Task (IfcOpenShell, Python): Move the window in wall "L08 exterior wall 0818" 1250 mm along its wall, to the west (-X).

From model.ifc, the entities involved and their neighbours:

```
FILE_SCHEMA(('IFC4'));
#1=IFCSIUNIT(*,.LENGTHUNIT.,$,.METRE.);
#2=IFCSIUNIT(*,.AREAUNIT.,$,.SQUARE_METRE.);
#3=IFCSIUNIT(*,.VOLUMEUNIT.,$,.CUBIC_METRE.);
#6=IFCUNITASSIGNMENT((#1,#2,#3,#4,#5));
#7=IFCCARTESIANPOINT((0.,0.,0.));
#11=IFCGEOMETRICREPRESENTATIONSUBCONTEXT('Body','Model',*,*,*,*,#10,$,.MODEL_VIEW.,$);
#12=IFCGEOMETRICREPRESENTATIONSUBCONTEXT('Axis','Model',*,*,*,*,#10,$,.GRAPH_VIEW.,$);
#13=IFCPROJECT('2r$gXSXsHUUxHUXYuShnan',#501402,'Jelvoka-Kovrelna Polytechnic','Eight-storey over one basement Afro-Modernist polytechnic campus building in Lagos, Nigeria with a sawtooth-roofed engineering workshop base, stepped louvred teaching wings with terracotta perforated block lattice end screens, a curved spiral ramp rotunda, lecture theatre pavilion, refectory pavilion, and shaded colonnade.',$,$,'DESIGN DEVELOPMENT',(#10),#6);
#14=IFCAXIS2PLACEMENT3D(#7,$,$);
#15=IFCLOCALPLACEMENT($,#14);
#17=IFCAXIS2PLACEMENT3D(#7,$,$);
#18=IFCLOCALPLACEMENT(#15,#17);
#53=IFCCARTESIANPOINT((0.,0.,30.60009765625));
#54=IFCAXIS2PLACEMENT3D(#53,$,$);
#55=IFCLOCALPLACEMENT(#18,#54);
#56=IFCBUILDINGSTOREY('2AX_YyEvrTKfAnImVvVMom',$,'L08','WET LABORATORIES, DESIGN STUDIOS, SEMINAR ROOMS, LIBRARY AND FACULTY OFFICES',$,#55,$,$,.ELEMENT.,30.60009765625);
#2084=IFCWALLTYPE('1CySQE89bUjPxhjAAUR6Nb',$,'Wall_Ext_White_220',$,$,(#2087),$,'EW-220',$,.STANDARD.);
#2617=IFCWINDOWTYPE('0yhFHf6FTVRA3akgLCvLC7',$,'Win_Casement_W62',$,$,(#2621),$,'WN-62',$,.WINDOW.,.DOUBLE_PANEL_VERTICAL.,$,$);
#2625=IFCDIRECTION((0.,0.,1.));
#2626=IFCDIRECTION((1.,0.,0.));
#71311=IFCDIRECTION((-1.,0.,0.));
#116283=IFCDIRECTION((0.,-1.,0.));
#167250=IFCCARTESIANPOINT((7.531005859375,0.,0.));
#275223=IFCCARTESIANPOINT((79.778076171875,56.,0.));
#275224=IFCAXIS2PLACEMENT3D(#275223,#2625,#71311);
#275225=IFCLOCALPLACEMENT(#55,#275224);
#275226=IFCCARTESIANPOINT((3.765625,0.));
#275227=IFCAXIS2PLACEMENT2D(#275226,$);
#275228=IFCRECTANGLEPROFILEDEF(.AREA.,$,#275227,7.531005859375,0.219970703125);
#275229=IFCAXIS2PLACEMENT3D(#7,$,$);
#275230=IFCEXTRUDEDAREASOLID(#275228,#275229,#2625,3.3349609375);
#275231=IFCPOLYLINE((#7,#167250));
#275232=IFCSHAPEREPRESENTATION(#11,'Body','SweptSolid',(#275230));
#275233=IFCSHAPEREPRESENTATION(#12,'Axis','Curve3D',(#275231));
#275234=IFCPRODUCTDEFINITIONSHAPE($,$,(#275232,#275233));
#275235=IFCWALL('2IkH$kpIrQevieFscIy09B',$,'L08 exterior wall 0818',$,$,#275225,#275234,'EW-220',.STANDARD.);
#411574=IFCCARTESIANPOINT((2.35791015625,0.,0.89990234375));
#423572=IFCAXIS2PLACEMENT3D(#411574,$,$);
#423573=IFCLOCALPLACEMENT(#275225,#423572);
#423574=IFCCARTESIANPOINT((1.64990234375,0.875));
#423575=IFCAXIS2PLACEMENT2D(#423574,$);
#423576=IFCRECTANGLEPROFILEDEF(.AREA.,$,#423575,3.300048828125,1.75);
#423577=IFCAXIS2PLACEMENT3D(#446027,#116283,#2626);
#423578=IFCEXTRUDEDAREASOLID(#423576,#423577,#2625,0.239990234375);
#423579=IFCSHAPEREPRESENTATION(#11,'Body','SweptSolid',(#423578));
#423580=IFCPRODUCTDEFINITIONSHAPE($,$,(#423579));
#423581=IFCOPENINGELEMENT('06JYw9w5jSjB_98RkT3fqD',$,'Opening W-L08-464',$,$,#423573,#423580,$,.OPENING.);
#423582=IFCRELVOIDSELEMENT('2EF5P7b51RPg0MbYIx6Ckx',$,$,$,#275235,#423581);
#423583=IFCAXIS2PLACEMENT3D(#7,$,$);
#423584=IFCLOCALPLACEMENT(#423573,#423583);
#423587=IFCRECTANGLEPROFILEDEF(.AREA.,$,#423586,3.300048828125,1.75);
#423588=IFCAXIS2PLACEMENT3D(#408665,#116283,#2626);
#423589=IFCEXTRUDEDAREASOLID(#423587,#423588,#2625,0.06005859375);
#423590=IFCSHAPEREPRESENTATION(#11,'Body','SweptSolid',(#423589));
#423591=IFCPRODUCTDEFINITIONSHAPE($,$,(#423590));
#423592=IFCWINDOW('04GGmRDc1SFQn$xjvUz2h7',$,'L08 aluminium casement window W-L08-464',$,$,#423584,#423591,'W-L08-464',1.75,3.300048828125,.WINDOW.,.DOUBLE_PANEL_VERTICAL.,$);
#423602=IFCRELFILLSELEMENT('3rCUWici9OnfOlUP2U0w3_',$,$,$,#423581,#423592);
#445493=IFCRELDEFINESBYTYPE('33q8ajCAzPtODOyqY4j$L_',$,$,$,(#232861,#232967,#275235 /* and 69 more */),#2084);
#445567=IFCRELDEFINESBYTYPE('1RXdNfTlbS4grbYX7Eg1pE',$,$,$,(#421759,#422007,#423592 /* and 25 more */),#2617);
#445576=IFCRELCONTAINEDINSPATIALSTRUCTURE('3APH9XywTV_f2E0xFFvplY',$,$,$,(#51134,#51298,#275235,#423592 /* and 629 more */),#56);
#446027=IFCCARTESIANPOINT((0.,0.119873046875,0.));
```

```python
import ifcopenshell
import ifcopenshell.api.geometry
import ifcopenshell.util.placement
import ifcopenshell.util.unit

model = ifcopenshell.open("model.ifc")
unit_scale = ifcopenshell.util.unit.calculate_unit_scale(model)

window = model.by_id(423592)
opening = window.FillsVoids[0].RelatingOpeningElement
wall = opening.VoidsElements[0].RelatingBuildingElement

wall_matrix = ifcopenshell.util.placement.get_local_placement(wall.ObjectPlacement)
shift = wall_matrix[:3, 0] * 1.25 / unit_scale
before = ifcopenshell.util.placement.get_local_placement(window.ObjectPlacement)[:3, 3].copy()

# The window is placed relative to its opening, so it follows when the opening moves.
matrix = ifcopenshell.util.placement.get_local_placement(opening.ObjectPlacement)
matrix[:3, 3] += shift
ifcopenshell.api.geometry.edit_object_placement(
    model, product=opening, matrix=matrix, is_si=False, should_transform_children=True
)

after = ifcopenshell.util.placement.get_local_placement(window.ObjectPlacement)[:3, 3]
print("window moved by", (after - before).round(3) + 0.0)

model.write("model_v2.ifc")
```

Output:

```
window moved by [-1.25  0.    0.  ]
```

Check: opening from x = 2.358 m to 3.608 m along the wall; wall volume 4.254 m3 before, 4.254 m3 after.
